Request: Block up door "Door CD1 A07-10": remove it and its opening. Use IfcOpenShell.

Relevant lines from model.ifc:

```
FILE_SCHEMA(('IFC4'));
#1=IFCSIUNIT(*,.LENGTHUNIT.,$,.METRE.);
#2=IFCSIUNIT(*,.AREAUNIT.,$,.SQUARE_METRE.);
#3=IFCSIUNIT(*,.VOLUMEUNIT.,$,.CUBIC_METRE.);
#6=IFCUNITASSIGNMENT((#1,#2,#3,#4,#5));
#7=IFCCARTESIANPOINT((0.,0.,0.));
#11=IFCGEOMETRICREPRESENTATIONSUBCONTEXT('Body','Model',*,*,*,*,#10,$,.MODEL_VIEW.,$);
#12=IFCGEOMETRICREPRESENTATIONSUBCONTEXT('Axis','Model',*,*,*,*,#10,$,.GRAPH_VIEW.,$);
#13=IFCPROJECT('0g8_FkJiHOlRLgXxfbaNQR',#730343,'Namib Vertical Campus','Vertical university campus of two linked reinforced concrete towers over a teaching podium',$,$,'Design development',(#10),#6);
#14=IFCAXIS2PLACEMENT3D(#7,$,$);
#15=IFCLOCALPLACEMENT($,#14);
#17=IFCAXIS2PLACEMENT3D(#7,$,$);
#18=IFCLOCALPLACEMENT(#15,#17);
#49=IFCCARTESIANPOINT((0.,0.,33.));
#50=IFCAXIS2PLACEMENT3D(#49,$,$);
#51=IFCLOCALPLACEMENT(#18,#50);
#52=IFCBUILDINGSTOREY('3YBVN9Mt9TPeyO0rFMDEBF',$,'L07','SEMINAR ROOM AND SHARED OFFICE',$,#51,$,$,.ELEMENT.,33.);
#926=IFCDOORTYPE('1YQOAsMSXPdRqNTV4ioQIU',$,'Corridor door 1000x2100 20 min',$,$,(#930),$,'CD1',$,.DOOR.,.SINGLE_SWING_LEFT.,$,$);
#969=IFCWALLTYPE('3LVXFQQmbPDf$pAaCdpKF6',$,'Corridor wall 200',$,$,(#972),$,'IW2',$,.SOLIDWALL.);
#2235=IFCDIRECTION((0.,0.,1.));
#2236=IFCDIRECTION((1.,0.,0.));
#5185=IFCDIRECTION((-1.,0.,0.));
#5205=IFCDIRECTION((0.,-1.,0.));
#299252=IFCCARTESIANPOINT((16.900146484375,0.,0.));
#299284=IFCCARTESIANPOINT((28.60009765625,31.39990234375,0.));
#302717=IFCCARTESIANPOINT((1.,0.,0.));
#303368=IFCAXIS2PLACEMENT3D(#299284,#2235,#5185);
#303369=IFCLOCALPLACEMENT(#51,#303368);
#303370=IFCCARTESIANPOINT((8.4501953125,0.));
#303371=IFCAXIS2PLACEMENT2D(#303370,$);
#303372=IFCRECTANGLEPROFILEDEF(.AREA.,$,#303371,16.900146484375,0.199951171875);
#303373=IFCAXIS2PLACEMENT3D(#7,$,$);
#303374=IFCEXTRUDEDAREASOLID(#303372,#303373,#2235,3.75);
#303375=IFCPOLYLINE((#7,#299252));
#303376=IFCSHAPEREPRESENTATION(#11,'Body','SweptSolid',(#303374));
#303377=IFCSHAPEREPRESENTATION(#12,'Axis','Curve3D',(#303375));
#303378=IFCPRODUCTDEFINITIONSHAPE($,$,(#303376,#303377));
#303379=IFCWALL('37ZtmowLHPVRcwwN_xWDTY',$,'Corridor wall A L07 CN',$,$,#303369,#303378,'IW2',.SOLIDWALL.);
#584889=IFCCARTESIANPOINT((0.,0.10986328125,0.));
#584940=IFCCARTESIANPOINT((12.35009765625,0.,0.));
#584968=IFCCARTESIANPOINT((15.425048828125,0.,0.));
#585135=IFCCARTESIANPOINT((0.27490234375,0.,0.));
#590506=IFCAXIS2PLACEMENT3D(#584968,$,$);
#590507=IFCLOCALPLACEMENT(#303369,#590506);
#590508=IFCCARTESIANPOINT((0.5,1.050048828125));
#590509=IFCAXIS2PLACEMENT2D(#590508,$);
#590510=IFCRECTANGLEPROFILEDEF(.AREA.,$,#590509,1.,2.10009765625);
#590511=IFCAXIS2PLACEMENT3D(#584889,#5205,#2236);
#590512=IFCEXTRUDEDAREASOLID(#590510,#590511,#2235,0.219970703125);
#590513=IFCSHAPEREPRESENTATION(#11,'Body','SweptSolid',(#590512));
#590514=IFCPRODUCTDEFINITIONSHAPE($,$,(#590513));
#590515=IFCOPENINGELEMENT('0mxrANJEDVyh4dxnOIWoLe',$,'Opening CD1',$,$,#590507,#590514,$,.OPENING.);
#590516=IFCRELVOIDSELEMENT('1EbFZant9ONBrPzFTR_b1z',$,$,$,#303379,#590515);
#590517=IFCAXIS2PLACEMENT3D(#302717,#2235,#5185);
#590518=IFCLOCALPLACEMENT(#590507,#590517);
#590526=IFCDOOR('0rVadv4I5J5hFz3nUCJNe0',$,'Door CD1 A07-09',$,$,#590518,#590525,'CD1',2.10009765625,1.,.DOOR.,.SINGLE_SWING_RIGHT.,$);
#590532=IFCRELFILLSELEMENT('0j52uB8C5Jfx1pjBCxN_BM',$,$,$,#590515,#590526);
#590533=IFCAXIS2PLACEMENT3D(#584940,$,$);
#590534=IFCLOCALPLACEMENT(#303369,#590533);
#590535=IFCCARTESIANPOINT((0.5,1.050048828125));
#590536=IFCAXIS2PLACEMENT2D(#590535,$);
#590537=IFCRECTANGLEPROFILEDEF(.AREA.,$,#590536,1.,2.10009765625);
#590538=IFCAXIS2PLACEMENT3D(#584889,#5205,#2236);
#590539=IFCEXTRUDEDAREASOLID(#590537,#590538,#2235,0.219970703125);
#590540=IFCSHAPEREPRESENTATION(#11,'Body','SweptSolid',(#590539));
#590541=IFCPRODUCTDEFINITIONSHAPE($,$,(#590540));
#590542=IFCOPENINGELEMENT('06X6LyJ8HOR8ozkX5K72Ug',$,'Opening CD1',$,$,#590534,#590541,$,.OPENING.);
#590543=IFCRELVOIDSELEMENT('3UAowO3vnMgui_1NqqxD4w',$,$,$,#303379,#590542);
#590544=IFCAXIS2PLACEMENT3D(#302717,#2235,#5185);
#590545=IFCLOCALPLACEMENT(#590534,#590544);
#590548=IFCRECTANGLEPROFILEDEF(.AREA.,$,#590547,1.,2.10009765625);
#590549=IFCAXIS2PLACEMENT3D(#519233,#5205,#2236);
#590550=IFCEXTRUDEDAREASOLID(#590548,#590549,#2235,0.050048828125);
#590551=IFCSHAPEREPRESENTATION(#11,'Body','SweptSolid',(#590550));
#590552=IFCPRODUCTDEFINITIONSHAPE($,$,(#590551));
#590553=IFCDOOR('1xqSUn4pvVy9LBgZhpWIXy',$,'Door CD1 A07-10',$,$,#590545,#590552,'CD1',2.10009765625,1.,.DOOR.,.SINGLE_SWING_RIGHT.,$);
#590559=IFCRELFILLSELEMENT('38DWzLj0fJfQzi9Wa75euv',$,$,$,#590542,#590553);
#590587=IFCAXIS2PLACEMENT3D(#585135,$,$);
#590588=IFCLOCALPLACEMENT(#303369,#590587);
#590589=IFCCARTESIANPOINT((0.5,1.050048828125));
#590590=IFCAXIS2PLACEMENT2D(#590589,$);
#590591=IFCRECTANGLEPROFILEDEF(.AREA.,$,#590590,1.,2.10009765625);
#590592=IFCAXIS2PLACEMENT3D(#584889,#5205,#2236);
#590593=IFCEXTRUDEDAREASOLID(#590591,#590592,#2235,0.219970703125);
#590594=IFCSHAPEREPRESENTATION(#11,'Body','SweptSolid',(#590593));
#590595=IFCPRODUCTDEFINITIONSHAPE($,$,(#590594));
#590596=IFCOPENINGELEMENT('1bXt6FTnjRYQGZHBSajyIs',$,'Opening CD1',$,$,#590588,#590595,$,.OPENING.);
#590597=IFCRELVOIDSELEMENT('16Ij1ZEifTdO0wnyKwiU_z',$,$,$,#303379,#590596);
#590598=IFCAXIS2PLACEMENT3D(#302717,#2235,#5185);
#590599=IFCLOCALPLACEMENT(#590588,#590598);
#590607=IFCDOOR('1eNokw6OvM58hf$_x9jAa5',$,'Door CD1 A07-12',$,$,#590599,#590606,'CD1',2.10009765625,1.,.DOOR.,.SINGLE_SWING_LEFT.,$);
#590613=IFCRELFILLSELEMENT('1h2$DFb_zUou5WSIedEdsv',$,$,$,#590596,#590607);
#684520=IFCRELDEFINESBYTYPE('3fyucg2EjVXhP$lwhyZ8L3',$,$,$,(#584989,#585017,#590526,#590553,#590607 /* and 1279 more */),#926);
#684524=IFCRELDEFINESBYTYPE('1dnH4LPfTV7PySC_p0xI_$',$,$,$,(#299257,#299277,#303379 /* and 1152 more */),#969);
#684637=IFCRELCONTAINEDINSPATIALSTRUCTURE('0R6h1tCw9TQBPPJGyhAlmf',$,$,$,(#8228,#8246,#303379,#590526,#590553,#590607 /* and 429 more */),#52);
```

```python
import ifcopenshell
import ifcopenshell.api.feature
import ifcopenshell.api.root
import ifcopenshell.geom
import ifcopenshell.util.shape

model = ifcopenshell.open("model.ifc")
settings = ifcopenshell.geom.settings()


def volume(element):
    """Net volume in cubic metres, openings subtracted."""
    shape = ifcopenshell.geom.create_shape(settings, element)
    return ifcopenshell.util.shape.get_volume(shape.geometry)


door = model.by_guid("1xqSUn4pvVy9LBgZhpWIXy")
opening = door.FillsVoids[0].RelatingOpeningElement
wall = opening.VoidsElements[0].RelatingBuildingElement
before = volume(wall)

ifcopenshell.api.root.remove_product(model, product=door)
ifcopenshell.api.feature.remove_feature(model, feature=opening)

after = volume(wall)

print(f"wall volume {before:.3f} -> {after:.3f} m3")

model.write("model_rev.ifc")
```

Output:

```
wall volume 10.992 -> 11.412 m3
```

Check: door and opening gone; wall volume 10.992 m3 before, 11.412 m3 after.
